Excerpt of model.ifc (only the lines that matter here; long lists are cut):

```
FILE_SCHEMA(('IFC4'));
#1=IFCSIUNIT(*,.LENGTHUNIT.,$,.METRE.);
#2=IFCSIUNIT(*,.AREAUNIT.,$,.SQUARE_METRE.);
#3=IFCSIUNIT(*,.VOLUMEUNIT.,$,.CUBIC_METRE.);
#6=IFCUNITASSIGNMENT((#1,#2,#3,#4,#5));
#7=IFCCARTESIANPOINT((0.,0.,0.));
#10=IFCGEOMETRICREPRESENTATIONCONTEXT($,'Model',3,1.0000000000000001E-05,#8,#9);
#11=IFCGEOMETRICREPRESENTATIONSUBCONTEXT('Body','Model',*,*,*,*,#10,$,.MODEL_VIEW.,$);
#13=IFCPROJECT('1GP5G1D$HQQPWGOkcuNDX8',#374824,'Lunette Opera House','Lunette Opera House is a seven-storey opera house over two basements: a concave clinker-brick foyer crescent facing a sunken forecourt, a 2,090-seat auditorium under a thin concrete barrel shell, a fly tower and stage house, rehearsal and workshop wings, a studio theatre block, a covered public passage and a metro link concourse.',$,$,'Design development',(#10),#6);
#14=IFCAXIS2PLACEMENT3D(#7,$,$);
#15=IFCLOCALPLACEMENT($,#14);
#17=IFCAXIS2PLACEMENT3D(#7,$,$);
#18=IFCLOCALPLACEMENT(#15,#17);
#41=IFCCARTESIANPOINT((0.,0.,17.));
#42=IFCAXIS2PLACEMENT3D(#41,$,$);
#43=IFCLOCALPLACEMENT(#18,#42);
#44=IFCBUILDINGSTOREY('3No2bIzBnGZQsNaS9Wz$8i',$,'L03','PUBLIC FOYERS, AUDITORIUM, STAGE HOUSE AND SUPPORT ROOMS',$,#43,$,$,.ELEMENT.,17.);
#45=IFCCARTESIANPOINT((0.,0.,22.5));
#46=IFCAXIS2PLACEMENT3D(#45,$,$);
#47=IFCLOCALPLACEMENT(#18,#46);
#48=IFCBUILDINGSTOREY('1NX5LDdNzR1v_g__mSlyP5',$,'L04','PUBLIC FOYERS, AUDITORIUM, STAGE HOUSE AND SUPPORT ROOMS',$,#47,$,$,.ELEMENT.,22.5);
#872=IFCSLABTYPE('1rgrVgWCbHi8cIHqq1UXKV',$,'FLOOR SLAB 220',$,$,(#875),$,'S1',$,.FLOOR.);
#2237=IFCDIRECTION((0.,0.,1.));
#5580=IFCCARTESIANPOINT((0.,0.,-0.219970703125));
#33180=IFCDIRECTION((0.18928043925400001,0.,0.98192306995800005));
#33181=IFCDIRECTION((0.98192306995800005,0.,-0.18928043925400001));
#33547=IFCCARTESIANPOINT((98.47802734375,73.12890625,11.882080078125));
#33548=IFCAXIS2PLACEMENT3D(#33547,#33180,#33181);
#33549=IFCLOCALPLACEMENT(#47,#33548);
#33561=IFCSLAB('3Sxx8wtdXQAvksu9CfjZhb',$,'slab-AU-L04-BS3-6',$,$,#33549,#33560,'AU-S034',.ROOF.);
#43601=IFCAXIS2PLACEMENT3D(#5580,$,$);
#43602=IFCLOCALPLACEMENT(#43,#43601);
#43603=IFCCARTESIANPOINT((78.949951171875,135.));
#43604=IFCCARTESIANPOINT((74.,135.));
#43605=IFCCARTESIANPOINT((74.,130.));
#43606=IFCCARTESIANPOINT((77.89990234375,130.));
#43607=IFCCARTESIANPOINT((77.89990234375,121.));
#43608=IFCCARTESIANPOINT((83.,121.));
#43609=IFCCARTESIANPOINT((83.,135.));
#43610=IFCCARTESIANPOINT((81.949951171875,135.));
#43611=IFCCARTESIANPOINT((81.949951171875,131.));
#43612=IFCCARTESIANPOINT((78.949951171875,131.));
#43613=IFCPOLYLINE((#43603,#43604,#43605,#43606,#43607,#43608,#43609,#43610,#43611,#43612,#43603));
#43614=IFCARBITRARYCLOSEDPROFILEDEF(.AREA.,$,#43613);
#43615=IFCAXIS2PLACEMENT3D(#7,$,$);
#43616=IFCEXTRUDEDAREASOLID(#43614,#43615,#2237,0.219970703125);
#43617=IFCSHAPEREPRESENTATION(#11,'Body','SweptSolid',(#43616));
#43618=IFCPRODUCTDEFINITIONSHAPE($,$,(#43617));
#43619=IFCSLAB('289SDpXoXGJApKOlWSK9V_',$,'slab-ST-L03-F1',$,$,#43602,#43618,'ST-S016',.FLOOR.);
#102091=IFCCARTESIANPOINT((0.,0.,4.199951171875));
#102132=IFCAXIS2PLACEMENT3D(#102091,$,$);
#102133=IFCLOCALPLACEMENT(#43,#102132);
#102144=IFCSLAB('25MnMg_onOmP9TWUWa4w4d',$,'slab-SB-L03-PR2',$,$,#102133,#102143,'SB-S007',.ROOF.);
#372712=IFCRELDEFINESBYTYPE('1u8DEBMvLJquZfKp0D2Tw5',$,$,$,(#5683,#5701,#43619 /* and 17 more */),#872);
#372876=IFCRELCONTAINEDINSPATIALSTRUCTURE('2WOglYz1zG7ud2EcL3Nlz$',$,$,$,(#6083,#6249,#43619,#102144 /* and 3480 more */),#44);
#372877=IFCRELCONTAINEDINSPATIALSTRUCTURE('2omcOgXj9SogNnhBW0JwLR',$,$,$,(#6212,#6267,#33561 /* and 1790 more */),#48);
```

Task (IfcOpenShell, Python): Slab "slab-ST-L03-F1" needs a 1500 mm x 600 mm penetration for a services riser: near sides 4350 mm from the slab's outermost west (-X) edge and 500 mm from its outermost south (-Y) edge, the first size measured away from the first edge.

```python
import numpy as np
import ifcopenshell
import ifcopenshell.api.feature
import ifcopenshell.api.geometry
import ifcopenshell.api.root
import ifcopenshell.geom
import ifcopenshell.util.placement
import ifcopenshell.util.representation
import ifcopenshell.util.shape
import ifcopenshell.util.unit

model = ifcopenshell.open("model.ifc")
unit_scale = ifcopenshell.util.unit.calculate_unit_scale(model)
settings = ifcopenshell.geom.settings()


def volume(element):
    """Net volume in cubic metres, openings subtracted."""
    shape = ifcopenshell.geom.create_shape(settings, element)
    return ifcopenshell.util.shape.get_volume(shape.geometry)


slab = model.by_id(43619)
before = volume(slab)

# Extent in the slab's own axes, in metres. The edges named are its -X and -Y sides.
slab_shape = ifcopenshell.geom.create_shape(settings, slab)
vertices = ifcopenshell.util.shape.get_vertices(slab_shape.geometry)
x_min, y_min, bottom = vertices.min(axis=0)
top = vertices[:, 2].max()

opening = ifcopenshell.api.root.create_entity(model, ifc_class="IfcOpeningElement", name="Services riser opening", predefined_type="OPENING")
context = ifcopenshell.util.representation.get_context(model, "Model", "Body", "MODEL_VIEW")
width, depth = 1.5, 0.6
outline = [(0.0, 0.0), (width, 0.0), (width, depth), (0.0, depth), (0.0, 0.0)]
# Overshoot both faces by 50 mm so the cut is clean.
shape = ifcopenshell.api.geometry.add_slab_representation(
    model, context=context, depth=top - bottom + 0.1, polyline=outline
)
ifcopenshell.api.geometry.assign_representation(model, product=opening, representation=shape)

matrix = ifcopenshell.util.placement.get_local_placement(slab.ObjectPlacement)
matrix[:, 3] = matrix @ np.append(np.array([x_min + 4.35, y_min + 0.5, bottom - 0.05]) / unit_scale, 1.0)
ifcopenshell.api.geometry.edit_object_placement(model, product=opening, matrix=matrix, is_si=False)
ifcopenshell.api.feature.add_feature(model, feature=opening, element=slab)

after = volume(slab)

print(f"slab volume {before:.3f} -> {after:.3f} m3")

model.write("model_edited.ifc")
```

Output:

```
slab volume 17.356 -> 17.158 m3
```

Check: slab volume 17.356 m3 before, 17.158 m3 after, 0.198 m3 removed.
